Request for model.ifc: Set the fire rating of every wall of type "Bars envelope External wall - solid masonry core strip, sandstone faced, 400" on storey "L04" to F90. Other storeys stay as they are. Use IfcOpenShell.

First a look at what the model holds.

```python
import ifcopenshell
import ifcopenshell.util.element

model = ifcopenshell.open("model.ifc")
print(model.schema)
storey = next(s for s in model.by_type("IfcBuildingStorey") if s.Name == "L04")
walls = [e for e in ifcopenshell.util.element.get_decomposition(storey) if e.is_a("IfcWall")]
seen = {}
for e in walls:
    element_type = ifcopenshell.util.element.get_type(e)
    key = (element_type.Name if element_type != e and element_type else None, ifcopenshell.util.element.get_pset(e, "Pset_WallCommon", "FireRating"))
    seen[key] = seen.get(key, 0) + 1
for (name, value), count in sorted(seen.items(), key=str):
    print(count, "x", name, "|", value)
```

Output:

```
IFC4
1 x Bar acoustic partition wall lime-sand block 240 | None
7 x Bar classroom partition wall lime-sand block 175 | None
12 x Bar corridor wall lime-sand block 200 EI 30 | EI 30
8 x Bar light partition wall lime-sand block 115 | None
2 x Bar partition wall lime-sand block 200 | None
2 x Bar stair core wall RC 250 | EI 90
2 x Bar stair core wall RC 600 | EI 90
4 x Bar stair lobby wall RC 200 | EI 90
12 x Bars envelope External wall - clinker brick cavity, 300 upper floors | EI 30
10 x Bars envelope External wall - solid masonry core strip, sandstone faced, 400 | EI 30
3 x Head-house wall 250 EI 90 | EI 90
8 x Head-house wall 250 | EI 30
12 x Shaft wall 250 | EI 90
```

```python
import ifcopenshell
import ifcopenshell.api.pset
import ifcopenshell.util.element

model = ifcopenshell.open("model.ifc")

storey = next(s for s in model.by_type("IfcBuildingStorey") if s.Name == "L04")
walls = [e for e in ifcopenshell.util.element.get_decomposition(storey) if e.is_a("IfcWall")]

count = 0
for e in walls:
    element_type = ifcopenshell.util.element.get_type(e)
    if element_type in (None, e) or element_type.Name != "Bars envelope External wall - solid masonry core strip, sandstone faced, 400":
        continue
    # add_pset returns the element's existing set when there is one.
    pset = ifcopenshell.api.pset.add_pset(model, product=e, name="Pset_WallCommon")
    ifcopenshell.api.pset.edit_pset(model, pset=pset, properties={"FireRating": "F90"})
    count += 1

print(count, "walls updated")

model.write("model-out.ifc")
```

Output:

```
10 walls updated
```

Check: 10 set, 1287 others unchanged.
